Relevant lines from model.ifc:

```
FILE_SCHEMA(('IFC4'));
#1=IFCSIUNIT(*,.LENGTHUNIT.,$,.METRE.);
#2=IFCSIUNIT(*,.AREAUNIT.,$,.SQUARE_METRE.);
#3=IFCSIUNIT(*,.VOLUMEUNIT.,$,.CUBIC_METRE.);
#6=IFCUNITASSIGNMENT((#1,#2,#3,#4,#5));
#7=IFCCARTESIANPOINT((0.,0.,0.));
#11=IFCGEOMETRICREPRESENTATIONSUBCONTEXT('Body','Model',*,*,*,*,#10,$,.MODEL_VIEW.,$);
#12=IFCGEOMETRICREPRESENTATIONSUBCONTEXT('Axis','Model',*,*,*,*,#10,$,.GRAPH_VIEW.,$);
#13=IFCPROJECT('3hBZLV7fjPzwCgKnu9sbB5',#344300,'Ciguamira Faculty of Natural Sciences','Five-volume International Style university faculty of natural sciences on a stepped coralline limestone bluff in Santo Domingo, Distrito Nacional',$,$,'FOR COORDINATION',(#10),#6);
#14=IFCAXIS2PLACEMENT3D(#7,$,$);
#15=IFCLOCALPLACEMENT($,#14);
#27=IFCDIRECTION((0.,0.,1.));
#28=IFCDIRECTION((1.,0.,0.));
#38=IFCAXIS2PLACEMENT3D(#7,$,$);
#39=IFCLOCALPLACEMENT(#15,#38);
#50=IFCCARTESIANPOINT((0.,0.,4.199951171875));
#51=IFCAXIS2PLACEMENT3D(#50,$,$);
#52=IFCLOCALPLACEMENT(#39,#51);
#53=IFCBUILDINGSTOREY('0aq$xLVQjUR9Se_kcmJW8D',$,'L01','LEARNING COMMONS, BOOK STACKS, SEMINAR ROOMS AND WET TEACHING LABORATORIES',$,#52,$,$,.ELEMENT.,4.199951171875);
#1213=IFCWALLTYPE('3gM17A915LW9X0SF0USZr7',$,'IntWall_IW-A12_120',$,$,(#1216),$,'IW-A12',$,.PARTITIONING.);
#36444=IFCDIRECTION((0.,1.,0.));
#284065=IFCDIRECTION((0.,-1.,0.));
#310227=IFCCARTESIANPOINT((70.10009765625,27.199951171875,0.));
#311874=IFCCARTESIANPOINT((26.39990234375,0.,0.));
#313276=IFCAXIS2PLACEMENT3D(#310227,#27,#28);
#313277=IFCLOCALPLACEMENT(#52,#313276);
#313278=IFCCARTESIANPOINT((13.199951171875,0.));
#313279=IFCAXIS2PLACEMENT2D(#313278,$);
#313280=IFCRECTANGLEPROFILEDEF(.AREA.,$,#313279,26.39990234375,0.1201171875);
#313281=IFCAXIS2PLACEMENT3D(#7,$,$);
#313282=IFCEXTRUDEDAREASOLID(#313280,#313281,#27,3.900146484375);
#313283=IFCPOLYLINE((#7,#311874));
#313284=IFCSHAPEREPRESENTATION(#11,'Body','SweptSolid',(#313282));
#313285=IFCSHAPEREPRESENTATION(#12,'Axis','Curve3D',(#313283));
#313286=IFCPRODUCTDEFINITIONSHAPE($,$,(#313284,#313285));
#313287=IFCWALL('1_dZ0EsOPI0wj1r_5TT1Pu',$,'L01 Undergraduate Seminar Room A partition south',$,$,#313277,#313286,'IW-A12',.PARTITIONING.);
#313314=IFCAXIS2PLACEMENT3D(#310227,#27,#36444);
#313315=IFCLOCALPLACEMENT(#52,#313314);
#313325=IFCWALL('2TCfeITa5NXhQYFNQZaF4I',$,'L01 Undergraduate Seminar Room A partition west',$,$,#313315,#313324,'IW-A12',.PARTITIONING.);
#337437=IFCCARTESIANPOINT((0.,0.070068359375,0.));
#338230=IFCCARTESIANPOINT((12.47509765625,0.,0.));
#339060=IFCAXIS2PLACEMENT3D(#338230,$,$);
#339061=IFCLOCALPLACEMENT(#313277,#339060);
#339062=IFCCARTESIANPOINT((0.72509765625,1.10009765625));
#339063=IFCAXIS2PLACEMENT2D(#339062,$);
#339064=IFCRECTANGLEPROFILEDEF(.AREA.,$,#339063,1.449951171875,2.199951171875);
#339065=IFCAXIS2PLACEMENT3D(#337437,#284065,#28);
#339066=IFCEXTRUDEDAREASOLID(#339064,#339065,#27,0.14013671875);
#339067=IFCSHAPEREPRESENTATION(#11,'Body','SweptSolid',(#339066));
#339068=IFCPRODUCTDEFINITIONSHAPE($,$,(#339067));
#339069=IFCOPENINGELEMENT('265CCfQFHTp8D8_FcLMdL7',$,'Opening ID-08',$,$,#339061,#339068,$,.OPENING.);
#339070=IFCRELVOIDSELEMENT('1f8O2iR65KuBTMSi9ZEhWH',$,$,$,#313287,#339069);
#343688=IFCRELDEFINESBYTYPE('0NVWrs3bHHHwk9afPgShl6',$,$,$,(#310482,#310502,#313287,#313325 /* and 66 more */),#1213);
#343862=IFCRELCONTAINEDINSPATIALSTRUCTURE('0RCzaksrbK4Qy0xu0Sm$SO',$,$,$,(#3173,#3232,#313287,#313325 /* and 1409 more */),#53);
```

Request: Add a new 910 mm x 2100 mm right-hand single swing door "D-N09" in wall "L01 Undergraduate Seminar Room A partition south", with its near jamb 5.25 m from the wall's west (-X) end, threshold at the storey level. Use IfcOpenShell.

```python
import numpy as np
import ifcopenshell
import ifcopenshell.api.feature
import ifcopenshell.api.geometry
import ifcopenshell.api.root
import ifcopenshell.api.spatial
import ifcopenshell.geom
import ifcopenshell.util.element
import ifcopenshell.util.placement
import ifcopenshell.util.representation
import ifcopenshell.util.shape
import ifcopenshell.util.unit

model = ifcopenshell.open("model.ifc")
unit_scale = ifcopenshell.util.unit.calculate_unit_scale(model)
settings = ifcopenshell.geom.settings()


def volume(element):
    """Net volume in cubic metres, openings subtracted."""
    shape = ifcopenshell.geom.create_shape(settings, element)
    return ifcopenshell.util.shape.get_volume(shape.geometry)


wall = model.by_guid("1_dZ0EsOPI0wj1r_5TT1Pu")
storey = ifcopenshell.util.element.get_container(wall, ifc_class="IfcBuildingStorey")
context = ifcopenshell.util.representation.get_context(model, "Model", "Body", "MODEL_VIEW")
before = volume(wall)

width, height, from_end, sill = 0.91, 2.1, 5.25, 0.0  # metres

# The wall runs along its own X axis, and the end named is its -X end.
wall_shape = ifcopenshell.geom.create_shape(settings, wall)
x, y, z = ifcopenshell.util.shape.get_vertices(wall_shape.geometry).T
start = x.min() + from_end
face, thickness = float(y.min()), float(y.max() - y.min())
wall_matrix = ifcopenshell.util.placement.get_local_placement(wall.ObjectPlacement)
level = ifcopenshell.util.placement.get_local_placement(storey.ObjectPlacement)[2, 3]


def in_wall(x, y):
    """Placement at x, y metres in the wall's axes, at sill height."""
    matrix = wall_matrix.copy()
    matrix[:, 3] = wall_matrix @ np.array([x / unit_scale, y / unit_scale, 0.0, 1.0])
    matrix[2, 3] = level + sill / unit_scale
    return matrix


# Opening: a box that overshoots both wall faces by 50 mm.
opening = ifcopenshell.api.root.create_entity(model, ifc_class="IfcOpeningElement", predefined_type="OPENING")
box = ifcopenshell.api.geometry.add_wall_representation(
    model, context=context, length=width, height=height, thickness=thickness + 0.1
)
ifcopenshell.api.geometry.assign_representation(model, product=opening, representation=box)
ifcopenshell.api.geometry.edit_object_placement(model, product=opening, matrix=in_wall(start, face - 0.05), is_si=False)
ifcopenshell.api.feature.add_feature(model, feature=opening, element=wall)

door = ifcopenshell.api.root.create_entity(model, ifc_class="IfcDoor", name="D-N09", predefined_type="DOOR")
door.OverallWidth, door.OverallHeight = width / unit_scale, height / unit_scale
door.OperationType = "SINGLE_SWING_RIGHT"
body = ifcopenshell.api.geometry.add_door_representation(
    model,
    context=context,
    overall_width=door.OverallWidth,
    overall_height=door.OverallHeight,
    operation_type="SINGLE_SWING_RIGHT",
    lining_properties={"LiningDepth": thickness / unit_scale, "ThresholdDepth": thickness / unit_scale},
)
ifcopenshell.api.geometry.assign_representation(model, product=door, representation=body)
ifcopenshell.api.spatial.assign_container(model, products=[door], relating_structure=storey)
ifcopenshell.api.feature.add_filling(model, opening=opening, element=door)

# The lining spans the wall, so the door starts at the wall face.
ifcopenshell.api.geometry.edit_object_placement(model, product=door, matrix=in_wall(start, face), is_si=False)

after = volume(wall)

print(f"wall volume {before:.3f} -> {after:.3f} m3")

model.write("model_updated.ifc")
```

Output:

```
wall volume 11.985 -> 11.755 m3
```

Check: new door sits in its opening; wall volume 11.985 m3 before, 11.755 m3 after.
